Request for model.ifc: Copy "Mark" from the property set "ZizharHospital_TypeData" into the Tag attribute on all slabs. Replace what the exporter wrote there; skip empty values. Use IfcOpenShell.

First a look at what the model holds.

```python
import ifcopenshell
import ifcopenshell.util.element

model = ifcopenshell.open("model.ifc")
print(model.schema)
slabs = model.by_type("IfcSlab")
print(len(slabs), "slabs")
for e in slabs[:8]:
    source = ifcopenshell.util.element.get_pset(e, "ZizharHospital_TypeData", "Mark")
    target = e.Tag
    print(e.id(), repr(source), repr(target), sep=" | ")
```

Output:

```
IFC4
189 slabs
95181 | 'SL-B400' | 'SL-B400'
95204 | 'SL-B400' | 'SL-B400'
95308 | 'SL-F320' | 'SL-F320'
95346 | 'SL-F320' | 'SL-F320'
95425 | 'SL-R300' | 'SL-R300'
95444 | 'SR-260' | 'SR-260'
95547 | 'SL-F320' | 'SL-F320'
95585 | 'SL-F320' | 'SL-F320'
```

```python
import ifcopenshell
import ifcopenshell.util.element

model = ifcopenshell.open("model.ifc")

count = 0
for e in model.by_type("IfcSlab"):
    value = ifcopenshell.util.element.get_pset(e, "ZizharHospital_TypeData", "Mark")
    current = e.Tag
    if not value or not value.strip() or current == value:
        continue
    e.Tag = value
    count += 1

print(count, "slabs updated")

model.write("model-out.ifc")
```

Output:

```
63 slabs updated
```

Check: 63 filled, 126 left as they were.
